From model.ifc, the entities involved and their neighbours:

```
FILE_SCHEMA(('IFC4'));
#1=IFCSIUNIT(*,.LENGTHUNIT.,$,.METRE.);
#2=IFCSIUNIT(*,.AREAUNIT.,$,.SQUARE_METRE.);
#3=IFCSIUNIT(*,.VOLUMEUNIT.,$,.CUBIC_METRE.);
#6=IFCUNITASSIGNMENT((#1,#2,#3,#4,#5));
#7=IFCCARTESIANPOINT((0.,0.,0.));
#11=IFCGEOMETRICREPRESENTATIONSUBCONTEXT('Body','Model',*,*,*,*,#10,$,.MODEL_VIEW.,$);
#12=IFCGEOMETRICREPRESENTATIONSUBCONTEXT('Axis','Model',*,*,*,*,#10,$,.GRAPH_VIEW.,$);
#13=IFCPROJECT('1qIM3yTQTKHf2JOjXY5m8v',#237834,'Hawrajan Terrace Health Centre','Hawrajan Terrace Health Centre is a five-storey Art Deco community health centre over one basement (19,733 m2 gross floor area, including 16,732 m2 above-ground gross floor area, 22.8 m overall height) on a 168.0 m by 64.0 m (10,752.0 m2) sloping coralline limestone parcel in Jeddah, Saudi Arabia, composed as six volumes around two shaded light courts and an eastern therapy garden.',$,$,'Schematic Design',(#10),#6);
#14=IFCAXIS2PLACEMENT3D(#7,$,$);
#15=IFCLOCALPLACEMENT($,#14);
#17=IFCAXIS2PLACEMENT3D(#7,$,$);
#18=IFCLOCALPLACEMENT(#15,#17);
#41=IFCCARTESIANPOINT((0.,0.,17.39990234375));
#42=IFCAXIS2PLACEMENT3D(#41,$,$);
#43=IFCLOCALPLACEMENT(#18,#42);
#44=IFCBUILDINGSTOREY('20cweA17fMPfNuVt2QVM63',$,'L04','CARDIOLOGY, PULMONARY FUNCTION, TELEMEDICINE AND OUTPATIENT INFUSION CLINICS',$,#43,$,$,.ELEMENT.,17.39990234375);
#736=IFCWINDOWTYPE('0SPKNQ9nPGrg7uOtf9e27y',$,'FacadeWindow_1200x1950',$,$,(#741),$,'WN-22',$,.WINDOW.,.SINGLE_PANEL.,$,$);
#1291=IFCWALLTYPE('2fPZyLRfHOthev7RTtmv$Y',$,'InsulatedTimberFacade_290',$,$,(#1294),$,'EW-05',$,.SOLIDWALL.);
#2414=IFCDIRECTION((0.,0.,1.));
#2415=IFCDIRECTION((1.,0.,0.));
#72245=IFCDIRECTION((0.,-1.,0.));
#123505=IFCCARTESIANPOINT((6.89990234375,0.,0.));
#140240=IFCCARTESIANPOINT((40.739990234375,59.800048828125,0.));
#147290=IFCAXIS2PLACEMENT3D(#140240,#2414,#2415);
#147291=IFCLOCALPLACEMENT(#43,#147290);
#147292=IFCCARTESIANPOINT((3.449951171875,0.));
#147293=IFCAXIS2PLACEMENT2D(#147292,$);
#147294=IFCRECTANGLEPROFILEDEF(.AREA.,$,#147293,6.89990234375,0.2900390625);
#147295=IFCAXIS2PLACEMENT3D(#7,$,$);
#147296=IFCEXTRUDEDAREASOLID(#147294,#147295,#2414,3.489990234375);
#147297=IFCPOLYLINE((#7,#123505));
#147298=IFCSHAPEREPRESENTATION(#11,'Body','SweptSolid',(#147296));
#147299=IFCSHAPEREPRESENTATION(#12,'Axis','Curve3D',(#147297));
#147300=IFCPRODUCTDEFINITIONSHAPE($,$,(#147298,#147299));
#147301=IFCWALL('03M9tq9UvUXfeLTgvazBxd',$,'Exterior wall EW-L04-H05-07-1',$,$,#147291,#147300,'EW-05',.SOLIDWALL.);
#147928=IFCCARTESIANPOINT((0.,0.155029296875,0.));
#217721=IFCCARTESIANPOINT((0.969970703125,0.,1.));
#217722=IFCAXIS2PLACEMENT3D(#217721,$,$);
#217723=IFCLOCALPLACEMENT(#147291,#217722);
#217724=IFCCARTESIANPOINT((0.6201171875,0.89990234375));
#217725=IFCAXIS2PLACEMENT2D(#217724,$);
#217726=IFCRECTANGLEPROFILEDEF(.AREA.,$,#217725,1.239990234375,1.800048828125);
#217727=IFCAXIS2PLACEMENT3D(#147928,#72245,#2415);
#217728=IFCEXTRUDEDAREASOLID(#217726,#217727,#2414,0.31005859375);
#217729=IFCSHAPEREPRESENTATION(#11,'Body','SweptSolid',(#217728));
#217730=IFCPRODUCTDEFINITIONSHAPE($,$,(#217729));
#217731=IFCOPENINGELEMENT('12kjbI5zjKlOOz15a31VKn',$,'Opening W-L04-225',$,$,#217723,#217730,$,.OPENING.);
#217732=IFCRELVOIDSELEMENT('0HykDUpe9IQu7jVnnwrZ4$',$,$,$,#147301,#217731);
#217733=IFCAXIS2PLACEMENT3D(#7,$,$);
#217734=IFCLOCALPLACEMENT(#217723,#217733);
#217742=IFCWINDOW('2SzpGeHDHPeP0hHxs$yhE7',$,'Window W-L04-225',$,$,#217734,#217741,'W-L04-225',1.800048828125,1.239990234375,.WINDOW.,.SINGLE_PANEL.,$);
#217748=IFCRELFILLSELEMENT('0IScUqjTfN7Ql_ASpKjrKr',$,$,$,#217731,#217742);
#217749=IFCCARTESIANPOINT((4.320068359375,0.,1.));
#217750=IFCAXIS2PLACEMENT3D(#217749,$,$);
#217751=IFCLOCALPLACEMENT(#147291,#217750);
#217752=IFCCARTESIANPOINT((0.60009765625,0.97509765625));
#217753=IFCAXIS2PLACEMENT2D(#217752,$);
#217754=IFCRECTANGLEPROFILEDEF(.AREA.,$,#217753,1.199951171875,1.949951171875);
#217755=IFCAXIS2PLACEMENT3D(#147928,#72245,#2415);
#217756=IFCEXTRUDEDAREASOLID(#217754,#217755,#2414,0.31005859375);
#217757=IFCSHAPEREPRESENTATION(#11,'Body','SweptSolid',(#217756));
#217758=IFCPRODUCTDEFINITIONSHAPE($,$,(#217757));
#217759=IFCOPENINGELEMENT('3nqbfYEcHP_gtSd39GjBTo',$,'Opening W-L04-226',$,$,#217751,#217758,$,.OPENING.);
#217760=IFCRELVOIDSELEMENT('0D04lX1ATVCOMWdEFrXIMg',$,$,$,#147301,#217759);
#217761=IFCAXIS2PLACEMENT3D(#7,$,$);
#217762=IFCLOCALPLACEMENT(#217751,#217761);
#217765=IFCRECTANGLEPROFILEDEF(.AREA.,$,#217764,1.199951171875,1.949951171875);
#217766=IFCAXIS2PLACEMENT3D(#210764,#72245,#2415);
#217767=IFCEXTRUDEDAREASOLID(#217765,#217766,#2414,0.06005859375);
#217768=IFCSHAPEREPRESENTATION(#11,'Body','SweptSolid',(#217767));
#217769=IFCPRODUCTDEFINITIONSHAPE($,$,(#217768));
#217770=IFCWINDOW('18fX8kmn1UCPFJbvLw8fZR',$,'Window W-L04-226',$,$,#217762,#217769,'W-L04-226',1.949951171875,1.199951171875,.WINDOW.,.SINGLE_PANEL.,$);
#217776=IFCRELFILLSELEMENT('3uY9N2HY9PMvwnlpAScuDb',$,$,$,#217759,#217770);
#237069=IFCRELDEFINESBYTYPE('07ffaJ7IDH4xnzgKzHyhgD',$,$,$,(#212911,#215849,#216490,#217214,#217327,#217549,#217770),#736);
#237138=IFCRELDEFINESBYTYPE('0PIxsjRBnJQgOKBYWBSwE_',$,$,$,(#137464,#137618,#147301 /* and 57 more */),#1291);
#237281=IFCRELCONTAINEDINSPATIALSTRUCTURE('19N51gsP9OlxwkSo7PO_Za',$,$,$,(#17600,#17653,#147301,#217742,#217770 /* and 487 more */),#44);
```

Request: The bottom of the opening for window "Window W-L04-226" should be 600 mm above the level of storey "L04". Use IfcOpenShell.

```python
import numpy as np
import ifcopenshell
import ifcopenshell.api.geometry
import ifcopenshell.geom
import ifcopenshell.util.element
import ifcopenshell.util.placement
import ifcopenshell.util.shape
import ifcopenshell.util.unit

model = ifcopenshell.open("model.ifc")
unit_scale = ifcopenshell.util.unit.calculate_unit_scale(model)

window = model.by_id(217770)
opening = window.FillsVoids[0].RelatingOpeningElement
storey = ifcopenshell.util.element.get_container(window, ifc_class="IfcBuildingStorey")
level = ifcopenshell.util.placement.get_local_placement(storey.ObjectPlacement)[2, 3]

# The opening's origin need not be at the sill, so measure its lowest point.
shape = ifcopenshell.geom.create_shape(ifcopenshell.geom.settings(), opening)
bottom = ifcopenshell.util.shape.get_shape_bottom_elevation(shape, shape.geometry) / unit_scale
dz = level + 0.6 - bottom

shift = np.array([0.0, 0.0, dz])
# The window is placed relative to its opening, so it follows when the opening moves.
matrix = ifcopenshell.util.placement.get_local_placement(opening.ObjectPlacement)
matrix[:3, 3] += shift
ifcopenshell.api.geometry.edit_object_placement(
    model, product=opening, matrix=matrix, is_si=False, should_transform_children=True
)

print(f"moved by {dz * unit_scale:+.3f} m")

model.write("model_v2.ifc")
```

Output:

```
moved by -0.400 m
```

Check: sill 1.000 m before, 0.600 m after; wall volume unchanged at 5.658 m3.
